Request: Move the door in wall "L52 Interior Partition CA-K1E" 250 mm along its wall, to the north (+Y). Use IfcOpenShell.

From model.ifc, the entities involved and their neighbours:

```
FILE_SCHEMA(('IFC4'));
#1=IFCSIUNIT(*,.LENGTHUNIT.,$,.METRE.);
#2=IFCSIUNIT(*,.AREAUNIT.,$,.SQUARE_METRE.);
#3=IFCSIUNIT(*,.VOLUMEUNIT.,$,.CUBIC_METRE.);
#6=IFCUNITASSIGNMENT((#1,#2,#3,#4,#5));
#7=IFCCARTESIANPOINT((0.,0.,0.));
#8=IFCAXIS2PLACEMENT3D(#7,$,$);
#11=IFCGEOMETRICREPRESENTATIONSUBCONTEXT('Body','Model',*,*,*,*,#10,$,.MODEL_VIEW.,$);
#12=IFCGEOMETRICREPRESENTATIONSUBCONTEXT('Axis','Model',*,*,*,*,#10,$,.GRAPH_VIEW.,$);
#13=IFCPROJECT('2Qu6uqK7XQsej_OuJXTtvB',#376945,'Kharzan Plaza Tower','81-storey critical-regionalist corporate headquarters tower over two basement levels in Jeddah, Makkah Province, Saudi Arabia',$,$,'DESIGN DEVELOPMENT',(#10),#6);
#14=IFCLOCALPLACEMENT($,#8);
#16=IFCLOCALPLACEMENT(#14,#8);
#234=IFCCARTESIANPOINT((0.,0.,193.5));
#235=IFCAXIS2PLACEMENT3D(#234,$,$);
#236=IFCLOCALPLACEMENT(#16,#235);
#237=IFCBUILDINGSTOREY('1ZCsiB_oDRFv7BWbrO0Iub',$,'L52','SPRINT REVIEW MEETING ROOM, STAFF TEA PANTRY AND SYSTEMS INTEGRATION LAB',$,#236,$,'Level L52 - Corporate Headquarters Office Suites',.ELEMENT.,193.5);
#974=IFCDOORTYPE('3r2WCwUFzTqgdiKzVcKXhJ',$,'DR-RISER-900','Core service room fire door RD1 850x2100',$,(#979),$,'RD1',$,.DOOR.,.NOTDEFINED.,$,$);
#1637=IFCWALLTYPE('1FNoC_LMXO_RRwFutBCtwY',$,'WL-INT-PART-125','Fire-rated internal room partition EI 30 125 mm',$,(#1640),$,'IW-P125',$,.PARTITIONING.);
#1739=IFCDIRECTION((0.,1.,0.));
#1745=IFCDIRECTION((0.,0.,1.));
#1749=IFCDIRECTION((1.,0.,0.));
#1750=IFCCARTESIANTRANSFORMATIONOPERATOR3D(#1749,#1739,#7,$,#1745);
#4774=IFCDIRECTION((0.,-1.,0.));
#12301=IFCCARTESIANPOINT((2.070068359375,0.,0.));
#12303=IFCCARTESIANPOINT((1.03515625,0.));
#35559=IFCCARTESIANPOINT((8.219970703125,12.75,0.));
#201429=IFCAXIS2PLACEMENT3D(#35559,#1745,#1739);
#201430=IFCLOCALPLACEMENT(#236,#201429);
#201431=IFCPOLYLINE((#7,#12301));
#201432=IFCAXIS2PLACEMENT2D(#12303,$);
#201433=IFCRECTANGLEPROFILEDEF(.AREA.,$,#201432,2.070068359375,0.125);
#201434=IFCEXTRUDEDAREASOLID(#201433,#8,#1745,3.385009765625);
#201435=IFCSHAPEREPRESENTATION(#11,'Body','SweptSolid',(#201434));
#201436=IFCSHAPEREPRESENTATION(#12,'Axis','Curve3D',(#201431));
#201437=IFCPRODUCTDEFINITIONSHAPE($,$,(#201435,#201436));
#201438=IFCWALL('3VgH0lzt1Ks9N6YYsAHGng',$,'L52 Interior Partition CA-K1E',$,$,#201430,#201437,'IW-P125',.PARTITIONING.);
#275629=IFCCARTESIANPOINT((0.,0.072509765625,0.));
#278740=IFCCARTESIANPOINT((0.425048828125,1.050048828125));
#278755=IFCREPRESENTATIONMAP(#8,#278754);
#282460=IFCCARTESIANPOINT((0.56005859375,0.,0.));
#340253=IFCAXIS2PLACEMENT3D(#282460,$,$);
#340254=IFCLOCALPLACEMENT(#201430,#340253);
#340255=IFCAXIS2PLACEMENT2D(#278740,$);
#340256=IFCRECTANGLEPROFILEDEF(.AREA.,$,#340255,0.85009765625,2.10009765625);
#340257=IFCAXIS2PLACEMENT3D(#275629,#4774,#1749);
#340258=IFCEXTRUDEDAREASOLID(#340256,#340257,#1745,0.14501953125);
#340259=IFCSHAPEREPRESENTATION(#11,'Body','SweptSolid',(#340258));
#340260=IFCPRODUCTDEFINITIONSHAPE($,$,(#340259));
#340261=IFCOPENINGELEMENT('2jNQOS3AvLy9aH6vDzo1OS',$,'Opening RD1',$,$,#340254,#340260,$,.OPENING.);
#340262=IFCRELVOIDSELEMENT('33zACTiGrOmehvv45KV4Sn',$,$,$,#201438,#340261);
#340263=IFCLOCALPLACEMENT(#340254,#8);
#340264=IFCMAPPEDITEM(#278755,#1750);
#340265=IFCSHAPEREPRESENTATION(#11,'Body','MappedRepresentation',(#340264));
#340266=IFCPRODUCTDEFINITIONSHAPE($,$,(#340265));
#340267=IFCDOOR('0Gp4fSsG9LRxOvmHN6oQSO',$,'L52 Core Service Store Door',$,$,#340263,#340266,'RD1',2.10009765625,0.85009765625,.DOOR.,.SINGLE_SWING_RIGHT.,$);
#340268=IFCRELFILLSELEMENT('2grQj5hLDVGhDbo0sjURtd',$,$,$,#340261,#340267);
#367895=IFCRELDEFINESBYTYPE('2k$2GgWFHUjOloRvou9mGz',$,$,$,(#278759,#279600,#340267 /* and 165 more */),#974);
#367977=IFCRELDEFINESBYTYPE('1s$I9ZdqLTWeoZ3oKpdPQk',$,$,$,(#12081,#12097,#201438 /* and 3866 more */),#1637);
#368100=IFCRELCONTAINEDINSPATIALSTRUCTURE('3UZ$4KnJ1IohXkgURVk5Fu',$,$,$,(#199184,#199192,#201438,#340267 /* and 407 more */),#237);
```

```python
import ifcopenshell
import ifcopenshell.api.geometry
import ifcopenshell.util.placement
import ifcopenshell.util.unit

model = ifcopenshell.open("model.ifc")
unit_scale = ifcopenshell.util.unit.calculate_unit_scale(model)

door = model.by_id(340267)
opening = door.FillsVoids[0].RelatingOpeningElement
wall = opening.VoidsElements[0].RelatingBuildingElement

wall_matrix = ifcopenshell.util.placement.get_local_placement(wall.ObjectPlacement)
shift = wall_matrix[:3, 0] * 0.25 / unit_scale
before = ifcopenshell.util.placement.get_local_placement(door.ObjectPlacement)[:3, 3].copy()

# The door is placed relative to its opening, so it follows when the opening moves.
matrix = ifcopenshell.util.placement.get_local_placement(opening.ObjectPlacement)
matrix[:3, 3] += shift
ifcopenshell.api.geometry.edit_object_placement(
    model, product=opening, matrix=matrix, is_si=False, should_transform_children=True
)

after = ifcopenshell.util.placement.get_local_placement(door.ObjectPlacement)[:3, 3]
print("door moved by", (after - before).round(3) + 0.0)

model.write("model_updated.ifc")
```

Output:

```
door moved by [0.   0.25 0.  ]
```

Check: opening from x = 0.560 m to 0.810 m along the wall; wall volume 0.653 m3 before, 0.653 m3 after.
